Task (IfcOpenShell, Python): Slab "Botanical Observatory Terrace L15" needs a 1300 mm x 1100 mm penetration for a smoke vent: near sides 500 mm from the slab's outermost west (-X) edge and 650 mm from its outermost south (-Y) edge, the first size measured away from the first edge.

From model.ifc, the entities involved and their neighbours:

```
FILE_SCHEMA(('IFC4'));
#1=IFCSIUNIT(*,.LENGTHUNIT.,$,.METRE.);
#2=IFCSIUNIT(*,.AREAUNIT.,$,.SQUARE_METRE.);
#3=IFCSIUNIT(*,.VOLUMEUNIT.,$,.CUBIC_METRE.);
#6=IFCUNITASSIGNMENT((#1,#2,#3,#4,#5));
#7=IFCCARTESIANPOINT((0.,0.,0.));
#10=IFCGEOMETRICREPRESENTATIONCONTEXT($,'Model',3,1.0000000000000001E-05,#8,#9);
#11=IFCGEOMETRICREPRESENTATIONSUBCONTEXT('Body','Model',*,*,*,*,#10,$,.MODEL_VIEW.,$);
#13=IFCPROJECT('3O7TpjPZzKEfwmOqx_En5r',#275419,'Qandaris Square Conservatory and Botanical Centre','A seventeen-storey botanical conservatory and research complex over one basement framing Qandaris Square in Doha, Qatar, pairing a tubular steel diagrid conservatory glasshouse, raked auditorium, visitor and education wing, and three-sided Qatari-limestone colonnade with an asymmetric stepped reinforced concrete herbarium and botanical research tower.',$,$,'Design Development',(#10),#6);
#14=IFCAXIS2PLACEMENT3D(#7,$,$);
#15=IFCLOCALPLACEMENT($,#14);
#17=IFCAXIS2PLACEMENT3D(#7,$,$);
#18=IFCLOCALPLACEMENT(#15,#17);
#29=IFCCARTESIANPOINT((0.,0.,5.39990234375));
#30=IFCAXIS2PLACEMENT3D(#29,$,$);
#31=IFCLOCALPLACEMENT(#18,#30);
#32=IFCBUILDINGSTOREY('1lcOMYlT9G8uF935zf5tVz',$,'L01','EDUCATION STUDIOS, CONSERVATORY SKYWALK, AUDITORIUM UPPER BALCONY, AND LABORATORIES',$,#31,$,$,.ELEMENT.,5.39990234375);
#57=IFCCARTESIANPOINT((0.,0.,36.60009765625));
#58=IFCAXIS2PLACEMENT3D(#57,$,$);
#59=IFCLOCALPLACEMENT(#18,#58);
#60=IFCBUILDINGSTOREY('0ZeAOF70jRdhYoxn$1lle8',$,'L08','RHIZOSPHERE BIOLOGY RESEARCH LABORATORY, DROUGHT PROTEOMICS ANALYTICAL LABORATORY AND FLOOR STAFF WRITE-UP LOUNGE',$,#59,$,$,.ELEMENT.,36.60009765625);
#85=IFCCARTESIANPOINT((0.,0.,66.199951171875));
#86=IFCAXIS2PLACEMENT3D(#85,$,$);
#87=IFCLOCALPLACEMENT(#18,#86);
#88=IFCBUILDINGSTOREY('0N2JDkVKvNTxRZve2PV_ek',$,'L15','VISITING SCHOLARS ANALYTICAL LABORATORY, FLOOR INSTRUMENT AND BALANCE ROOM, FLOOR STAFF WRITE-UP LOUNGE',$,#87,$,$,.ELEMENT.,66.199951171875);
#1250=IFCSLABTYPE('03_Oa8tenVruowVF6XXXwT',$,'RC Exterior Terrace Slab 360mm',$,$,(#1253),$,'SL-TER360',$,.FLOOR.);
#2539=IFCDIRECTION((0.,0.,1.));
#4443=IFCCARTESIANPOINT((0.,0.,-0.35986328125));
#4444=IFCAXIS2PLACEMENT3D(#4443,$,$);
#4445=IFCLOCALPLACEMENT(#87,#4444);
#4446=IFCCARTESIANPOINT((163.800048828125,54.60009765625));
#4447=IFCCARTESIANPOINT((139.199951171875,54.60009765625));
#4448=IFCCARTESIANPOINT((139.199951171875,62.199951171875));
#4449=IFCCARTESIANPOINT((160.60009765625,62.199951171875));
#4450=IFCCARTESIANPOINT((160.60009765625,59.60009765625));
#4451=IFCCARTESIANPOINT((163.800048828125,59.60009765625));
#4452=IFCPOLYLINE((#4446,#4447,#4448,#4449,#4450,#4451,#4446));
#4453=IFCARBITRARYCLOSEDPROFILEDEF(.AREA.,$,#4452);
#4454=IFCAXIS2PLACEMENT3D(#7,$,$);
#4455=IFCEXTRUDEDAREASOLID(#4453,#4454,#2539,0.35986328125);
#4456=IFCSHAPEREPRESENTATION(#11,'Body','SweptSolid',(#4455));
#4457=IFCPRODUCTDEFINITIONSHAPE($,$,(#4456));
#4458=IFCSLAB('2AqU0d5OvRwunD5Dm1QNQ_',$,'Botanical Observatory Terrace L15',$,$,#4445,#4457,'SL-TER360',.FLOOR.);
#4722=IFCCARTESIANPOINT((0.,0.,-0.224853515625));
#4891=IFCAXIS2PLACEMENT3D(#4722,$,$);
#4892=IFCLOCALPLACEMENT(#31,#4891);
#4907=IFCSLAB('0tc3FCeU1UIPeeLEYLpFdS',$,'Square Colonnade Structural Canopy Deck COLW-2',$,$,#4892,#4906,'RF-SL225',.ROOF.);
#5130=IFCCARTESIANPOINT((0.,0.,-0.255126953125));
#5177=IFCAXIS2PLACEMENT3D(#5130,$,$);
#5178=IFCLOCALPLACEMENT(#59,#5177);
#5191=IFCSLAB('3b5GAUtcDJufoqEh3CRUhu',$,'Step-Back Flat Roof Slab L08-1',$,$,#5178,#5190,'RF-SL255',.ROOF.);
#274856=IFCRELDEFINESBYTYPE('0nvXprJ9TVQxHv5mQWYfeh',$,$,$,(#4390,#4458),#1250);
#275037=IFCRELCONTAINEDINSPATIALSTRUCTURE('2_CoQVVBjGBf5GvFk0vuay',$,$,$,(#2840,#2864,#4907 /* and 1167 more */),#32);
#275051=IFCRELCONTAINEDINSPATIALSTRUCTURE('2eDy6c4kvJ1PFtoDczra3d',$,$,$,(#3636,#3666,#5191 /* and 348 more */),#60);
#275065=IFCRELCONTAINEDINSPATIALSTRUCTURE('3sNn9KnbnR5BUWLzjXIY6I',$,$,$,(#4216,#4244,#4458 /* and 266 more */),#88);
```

```python
import numpy as np
import ifcopenshell
import ifcopenshell.api.feature
import ifcopenshell.api.geometry
import ifcopenshell.api.root
import ifcopenshell.geom
import ifcopenshell.util.placement
import ifcopenshell.util.representation
import ifcopenshell.util.shape
import ifcopenshell.util.unit

model = ifcopenshell.open("model.ifc")
unit_scale = ifcopenshell.util.unit.calculate_unit_scale(model)
settings = ifcopenshell.geom.settings()


def volume(element):
    """Net volume in cubic metres, openings subtracted."""
    shape = ifcopenshell.geom.create_shape(settings, element)
    return ifcopenshell.util.shape.get_volume(shape.geometry)


slab = model.by_guid("2AqU0d5OvRwunD5Dm1QNQ_")
before = volume(slab)

# Extent in the slab's own axes, in metres. The edges named are its -X and -Y sides.
slab_shape = ifcopenshell.geom.create_shape(settings, slab)
vertices = ifcopenshell.util.shape.get_vertices(slab_shape.geometry)
x_min, y_min, bottom = vertices.min(axis=0)
top = vertices[:, 2].max()

opening = ifcopenshell.api.root.create_entity(model, ifc_class="IfcOpeningElement", name="Smoke vent opening", predefined_type="OPENING")
context = ifcopenshell.util.representation.get_context(model, "Model", "Body", "MODEL_VIEW")
width, depth = 1.3, 1.1
outline = [(0.0, 0.0), (width, 0.0), (width, depth), (0.0, depth), (0.0, 0.0)]
# Overshoot both faces by 50 mm so the cut is clean.
shape = ifcopenshell.api.geometry.add_slab_representation(
    model, context=context, depth=top - bottom + 0.1, polyline=outline
)
ifcopenshell.api.geometry.assign_representation(model, product=opening, representation=shape)

matrix = ifcopenshell.util.placement.get_local_placement(slab.ObjectPlacement)
matrix[:, 3] = matrix @ np.append(np.array([x_min + 0.5, y_min + 0.65, bottom - 0.05]) / unit_scale, 1.0)
ifcopenshell.api.geometry.edit_object_placement(model, product=opening, matrix=matrix, is_si=False)
ifcopenshell.api.feature.add_feature(model, feature=opening, element=slab)

after = volume(slab)

print(f"slab volume {before:.3f} -> {after:.3f} m3")

model.write("model_edited.ifc")
```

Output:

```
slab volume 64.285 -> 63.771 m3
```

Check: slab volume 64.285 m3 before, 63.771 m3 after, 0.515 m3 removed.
